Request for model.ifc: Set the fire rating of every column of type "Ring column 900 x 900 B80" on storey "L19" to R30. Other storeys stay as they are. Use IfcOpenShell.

First a look at what the model holds.

```python
import ifcopenshell
import ifcopenshell.util.element

model = ifcopenshell.open("model.ifc")
print(model.schema)
storey = next(s for s in model.by_type("IfcBuildingStorey") if s.Name == "L19")
columns = [e for e in ifcopenshell.util.element.get_decomposition(storey) if e.is_a("IfcColumn")]
seen = {}
for e in columns:
    element_type = ifcopenshell.util.element.get_type(e)
    key = (element_type.Name if element_type != e and element_type else None, ifcopenshell.util.element.get_pset(e, "Pset_ColumnCommon", "FireRating"))
    seen[key] = seen.get(key, 0) + 1
for (name, value), count in sorted(seen.items(), key=str):
    print(count, "x", name, "|", value)
```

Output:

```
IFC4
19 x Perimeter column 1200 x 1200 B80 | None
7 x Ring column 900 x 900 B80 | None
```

```python
import ifcopenshell
import ifcopenshell.api.pset
import ifcopenshell.util.element

model = ifcopenshell.open("model.ifc")

storey = next(s for s in model.by_type("IfcBuildingStorey") if s.Name == "L19")
columns = [e for e in ifcopenshell.util.element.get_decomposition(storey) if e.is_a("IfcColumn")]

count = 0
for e in columns:
    element_type = ifcopenshell.util.element.get_type(e)
    if element_type in (None, e) or element_type.Name != "Ring column 900 x 900 B80":
        continue
    found = ifcopenshell.util.element.get_pset(e, "Pset_ColumnCommon", should_inherit=False)
    if found:
        pset = model.by_id(found["id"])
        if len(ifcopenshell.util.element.get_elements_by_pset(pset)) > 1:
            pset = ifcopenshell.api.pset.unshare_pset(model, products=[e], pset=pset)[0]
    else:
        pset = ifcopenshell.api.pset.add_pset(model, product=e, name="Pset_ColumnCommon")
    ifcopenshell.api.pset.edit_pset(model, pset=pset, properties={"FireRating": "R30"})
    count += 1

print(count, "columns updated")

model.write("model_updated.ifc")
```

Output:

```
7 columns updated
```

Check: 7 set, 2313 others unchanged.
